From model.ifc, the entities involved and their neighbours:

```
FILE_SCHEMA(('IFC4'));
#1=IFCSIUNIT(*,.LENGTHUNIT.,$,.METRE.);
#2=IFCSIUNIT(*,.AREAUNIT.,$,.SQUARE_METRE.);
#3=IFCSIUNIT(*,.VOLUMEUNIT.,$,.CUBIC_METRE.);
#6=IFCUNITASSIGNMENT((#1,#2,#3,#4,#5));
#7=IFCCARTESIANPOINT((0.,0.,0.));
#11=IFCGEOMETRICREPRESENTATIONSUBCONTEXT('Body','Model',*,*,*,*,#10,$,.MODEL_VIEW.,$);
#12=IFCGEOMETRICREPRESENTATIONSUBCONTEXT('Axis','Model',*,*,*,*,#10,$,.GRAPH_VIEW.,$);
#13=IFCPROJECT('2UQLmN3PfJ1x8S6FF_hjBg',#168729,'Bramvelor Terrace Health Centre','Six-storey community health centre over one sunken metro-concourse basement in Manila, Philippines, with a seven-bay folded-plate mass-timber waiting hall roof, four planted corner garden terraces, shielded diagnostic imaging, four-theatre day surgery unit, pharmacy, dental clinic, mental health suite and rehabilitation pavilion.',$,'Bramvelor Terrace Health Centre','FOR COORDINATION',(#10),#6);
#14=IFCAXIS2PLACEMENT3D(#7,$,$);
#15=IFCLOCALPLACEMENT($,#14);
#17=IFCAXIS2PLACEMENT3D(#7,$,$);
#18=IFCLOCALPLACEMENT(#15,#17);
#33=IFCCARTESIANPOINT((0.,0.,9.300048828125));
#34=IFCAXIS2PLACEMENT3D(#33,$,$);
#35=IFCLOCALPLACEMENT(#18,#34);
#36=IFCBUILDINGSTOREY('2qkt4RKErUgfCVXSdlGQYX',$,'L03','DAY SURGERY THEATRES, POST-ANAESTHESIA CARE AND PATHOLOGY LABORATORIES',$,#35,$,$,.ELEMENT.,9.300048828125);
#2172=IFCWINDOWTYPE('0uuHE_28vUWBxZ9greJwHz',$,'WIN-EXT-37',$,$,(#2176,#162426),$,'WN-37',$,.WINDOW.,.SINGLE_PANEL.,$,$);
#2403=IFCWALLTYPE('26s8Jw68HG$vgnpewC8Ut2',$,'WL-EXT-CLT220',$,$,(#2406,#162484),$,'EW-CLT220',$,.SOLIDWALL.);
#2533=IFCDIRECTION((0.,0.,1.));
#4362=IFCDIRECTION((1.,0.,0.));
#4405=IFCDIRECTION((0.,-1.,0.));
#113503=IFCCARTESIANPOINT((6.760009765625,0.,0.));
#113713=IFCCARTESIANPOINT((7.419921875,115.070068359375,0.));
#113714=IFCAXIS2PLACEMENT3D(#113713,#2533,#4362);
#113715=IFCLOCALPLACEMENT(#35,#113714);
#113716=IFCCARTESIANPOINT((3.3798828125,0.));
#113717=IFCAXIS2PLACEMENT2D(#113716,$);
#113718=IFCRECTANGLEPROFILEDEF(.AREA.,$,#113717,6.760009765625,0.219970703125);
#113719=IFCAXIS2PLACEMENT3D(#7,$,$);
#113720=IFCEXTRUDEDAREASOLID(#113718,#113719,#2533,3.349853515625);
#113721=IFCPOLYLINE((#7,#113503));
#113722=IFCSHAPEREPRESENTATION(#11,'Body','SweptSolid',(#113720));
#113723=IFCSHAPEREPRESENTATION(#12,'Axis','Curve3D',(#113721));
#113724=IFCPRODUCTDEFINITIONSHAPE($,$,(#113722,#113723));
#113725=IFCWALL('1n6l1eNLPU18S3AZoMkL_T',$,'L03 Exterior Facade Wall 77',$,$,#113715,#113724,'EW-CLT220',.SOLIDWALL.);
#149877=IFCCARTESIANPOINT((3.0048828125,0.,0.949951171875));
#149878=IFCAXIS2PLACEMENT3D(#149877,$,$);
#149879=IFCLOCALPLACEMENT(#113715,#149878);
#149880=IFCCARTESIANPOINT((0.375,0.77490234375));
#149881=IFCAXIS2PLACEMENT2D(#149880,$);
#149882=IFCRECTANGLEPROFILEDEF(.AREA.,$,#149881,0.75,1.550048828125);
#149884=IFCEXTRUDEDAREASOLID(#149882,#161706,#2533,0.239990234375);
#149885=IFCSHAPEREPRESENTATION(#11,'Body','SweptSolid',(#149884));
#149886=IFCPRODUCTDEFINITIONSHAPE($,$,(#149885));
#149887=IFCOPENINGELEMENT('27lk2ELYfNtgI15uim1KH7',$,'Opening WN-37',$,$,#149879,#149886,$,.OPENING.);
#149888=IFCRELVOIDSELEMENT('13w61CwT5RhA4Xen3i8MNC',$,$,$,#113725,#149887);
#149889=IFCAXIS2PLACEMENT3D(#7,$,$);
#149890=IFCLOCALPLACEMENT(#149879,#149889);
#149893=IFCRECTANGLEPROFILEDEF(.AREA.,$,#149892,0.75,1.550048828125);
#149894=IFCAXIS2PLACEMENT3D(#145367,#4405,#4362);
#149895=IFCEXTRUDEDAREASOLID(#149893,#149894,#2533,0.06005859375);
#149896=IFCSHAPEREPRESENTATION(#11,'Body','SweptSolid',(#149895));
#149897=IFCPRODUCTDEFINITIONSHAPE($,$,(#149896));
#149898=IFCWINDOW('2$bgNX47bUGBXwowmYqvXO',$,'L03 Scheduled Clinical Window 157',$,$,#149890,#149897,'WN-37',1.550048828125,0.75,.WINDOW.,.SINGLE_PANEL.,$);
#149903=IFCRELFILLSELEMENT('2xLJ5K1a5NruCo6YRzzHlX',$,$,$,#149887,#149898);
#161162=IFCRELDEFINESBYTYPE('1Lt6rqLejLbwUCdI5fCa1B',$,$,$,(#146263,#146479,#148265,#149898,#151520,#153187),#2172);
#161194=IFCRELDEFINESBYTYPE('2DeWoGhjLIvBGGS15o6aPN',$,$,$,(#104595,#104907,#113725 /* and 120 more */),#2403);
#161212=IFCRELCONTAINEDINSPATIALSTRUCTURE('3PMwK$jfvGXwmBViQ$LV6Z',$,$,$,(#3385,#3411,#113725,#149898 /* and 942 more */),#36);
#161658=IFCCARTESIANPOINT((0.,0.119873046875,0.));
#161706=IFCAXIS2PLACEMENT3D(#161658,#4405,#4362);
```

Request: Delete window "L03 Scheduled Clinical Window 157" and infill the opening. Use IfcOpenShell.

```python
import ifcopenshell
import ifcopenshell.api.feature
import ifcopenshell.api.root
import ifcopenshell.geom
import ifcopenshell.util.shape

model = ifcopenshell.open("model.ifc")
settings = ifcopenshell.geom.settings()


def volume(element):
    """Net volume in cubic metres, openings subtracted."""
    shape = ifcopenshell.geom.create_shape(settings, element)
    return ifcopenshell.util.shape.get_volume(shape.geometry)


window = model.by_guid("2$bgNX47bUGBXwowmYqvXO")
opening = window.FillsVoids[0].RelatingOpeningElement
wall = opening.VoidsElements[0].RelatingBuildingElement
before = volume(wall)

ifcopenshell.api.root.remove_product(model, product=window)
ifcopenshell.api.feature.remove_feature(model, feature=opening)

after = volume(wall)

print(f"wall volume {before:.3f} -> {after:.3f} m3")

model.write("model_v2.ifc")
```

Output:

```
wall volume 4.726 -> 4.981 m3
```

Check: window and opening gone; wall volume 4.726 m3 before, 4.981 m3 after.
